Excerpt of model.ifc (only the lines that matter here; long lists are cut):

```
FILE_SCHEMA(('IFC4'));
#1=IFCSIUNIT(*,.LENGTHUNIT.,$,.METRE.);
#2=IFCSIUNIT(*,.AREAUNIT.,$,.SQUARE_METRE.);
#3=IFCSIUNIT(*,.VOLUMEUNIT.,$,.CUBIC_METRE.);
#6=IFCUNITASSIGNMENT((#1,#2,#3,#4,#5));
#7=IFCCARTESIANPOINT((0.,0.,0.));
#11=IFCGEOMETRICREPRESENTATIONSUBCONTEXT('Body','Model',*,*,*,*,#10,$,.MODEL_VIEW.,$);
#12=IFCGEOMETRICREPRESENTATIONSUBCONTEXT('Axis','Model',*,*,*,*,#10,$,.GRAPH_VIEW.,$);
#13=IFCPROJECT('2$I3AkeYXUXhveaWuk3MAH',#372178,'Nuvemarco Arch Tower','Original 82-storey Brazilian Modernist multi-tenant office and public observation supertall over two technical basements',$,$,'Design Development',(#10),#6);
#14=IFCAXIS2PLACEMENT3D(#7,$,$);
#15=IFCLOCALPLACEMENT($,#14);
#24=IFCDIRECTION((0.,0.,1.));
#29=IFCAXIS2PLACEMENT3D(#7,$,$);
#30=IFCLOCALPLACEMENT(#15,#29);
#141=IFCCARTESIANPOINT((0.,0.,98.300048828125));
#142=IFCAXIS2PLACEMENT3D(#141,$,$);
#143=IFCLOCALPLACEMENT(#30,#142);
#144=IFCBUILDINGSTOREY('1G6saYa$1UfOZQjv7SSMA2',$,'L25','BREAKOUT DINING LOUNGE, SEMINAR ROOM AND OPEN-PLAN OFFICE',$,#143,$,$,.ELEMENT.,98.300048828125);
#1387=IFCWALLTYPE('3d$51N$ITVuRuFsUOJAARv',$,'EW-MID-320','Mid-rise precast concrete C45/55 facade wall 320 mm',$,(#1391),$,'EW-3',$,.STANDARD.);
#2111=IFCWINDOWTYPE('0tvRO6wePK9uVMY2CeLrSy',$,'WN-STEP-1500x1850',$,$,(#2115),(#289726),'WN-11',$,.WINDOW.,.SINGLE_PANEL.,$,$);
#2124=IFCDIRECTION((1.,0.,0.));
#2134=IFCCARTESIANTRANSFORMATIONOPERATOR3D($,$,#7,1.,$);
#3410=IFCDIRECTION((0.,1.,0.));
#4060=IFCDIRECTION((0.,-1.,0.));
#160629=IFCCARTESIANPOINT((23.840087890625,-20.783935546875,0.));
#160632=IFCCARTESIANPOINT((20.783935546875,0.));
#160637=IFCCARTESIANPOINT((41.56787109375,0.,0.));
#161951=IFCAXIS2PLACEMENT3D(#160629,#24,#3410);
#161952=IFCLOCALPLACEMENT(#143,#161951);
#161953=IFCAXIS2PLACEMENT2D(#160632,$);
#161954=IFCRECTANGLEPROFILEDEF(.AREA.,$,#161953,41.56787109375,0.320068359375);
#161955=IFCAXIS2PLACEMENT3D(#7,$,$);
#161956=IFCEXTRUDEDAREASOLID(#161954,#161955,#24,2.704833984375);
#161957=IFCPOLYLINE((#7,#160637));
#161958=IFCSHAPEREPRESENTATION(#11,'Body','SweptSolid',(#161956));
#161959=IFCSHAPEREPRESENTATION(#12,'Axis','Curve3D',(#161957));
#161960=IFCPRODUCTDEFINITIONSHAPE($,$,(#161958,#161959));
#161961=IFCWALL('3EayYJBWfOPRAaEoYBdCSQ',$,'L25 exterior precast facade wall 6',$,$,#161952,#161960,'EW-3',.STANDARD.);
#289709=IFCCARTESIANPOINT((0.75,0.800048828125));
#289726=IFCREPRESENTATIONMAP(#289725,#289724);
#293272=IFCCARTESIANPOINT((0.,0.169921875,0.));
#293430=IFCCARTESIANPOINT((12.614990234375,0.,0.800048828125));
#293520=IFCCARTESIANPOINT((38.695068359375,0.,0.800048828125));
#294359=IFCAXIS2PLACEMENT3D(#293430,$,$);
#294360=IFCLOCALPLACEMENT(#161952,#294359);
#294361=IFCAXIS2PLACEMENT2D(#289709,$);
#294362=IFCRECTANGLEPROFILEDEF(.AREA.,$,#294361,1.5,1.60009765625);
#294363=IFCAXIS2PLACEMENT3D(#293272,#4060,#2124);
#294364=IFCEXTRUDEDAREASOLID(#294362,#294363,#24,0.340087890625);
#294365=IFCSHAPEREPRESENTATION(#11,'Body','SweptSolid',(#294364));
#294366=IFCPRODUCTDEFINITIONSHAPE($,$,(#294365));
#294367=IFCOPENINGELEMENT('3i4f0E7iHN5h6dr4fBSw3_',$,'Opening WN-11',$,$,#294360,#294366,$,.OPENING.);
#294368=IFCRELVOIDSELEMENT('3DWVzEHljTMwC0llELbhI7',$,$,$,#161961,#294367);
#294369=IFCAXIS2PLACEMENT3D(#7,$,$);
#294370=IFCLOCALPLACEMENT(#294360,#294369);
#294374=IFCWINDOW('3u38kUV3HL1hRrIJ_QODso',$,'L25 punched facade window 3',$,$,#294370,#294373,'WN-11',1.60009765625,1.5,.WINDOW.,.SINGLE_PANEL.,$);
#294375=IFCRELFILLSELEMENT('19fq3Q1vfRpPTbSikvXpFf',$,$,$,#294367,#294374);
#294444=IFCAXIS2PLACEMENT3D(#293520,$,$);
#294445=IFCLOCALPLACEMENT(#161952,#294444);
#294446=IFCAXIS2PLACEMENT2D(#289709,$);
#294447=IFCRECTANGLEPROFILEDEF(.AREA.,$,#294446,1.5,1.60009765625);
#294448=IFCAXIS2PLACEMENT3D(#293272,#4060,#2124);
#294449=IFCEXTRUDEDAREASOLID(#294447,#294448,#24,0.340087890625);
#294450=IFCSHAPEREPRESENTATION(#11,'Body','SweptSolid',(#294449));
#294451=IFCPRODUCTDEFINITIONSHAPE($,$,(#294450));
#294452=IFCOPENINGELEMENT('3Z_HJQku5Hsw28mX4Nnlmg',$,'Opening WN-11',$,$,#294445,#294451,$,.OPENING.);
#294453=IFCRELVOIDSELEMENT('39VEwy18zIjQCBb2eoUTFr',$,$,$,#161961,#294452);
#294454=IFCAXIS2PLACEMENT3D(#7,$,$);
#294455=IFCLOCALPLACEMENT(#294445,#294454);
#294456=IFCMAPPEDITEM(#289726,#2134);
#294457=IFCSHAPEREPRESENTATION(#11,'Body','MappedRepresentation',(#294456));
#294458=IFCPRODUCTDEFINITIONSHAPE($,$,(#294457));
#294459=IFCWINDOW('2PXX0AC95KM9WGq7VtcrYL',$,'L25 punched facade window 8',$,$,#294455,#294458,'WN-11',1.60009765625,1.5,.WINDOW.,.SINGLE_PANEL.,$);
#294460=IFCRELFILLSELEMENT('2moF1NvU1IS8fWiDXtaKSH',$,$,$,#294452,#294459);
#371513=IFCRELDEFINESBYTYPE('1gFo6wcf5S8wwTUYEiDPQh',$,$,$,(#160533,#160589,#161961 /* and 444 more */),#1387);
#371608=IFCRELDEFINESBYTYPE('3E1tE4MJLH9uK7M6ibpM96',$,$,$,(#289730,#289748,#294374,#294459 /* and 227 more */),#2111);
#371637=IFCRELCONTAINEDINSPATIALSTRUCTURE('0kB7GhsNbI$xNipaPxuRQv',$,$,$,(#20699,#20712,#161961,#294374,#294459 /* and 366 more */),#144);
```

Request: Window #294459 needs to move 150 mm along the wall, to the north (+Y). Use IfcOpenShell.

```python
import ifcopenshell
import ifcopenshell.api.geometry
import ifcopenshell.util.placement

model = ifcopenshell.open("model.ifc")

window = model.by_id(294459)
opening = window.FillsVoids[0].RelatingOpeningElement
wall = opening.VoidsElements[0].RelatingBuildingElement

wall_matrix = ifcopenshell.util.placement.get_local_placement(wall.ObjectPlacement)
shift = wall_matrix[:3, 0] * 0.15
before = ifcopenshell.util.placement.get_local_placement(window.ObjectPlacement)[:3, 3].copy()

# The window is placed relative to its opening, so it follows when the opening moves.
matrix = ifcopenshell.util.placement.get_local_placement(opening.ObjectPlacement)
matrix[:3, 3] += shift
ifcopenshell.api.geometry.edit_object_placement(
    model, product=opening, matrix=matrix, is_si=False, should_transform_children=True
)

after = ifcopenshell.util.placement.get_local_placement(window.ObjectPlacement)[:3, 3]
print("window moved by", (after - before).round(3) + 0.0)

model.write("model-out.ifc")
```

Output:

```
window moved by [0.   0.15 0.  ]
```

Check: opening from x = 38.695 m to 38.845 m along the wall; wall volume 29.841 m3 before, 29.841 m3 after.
